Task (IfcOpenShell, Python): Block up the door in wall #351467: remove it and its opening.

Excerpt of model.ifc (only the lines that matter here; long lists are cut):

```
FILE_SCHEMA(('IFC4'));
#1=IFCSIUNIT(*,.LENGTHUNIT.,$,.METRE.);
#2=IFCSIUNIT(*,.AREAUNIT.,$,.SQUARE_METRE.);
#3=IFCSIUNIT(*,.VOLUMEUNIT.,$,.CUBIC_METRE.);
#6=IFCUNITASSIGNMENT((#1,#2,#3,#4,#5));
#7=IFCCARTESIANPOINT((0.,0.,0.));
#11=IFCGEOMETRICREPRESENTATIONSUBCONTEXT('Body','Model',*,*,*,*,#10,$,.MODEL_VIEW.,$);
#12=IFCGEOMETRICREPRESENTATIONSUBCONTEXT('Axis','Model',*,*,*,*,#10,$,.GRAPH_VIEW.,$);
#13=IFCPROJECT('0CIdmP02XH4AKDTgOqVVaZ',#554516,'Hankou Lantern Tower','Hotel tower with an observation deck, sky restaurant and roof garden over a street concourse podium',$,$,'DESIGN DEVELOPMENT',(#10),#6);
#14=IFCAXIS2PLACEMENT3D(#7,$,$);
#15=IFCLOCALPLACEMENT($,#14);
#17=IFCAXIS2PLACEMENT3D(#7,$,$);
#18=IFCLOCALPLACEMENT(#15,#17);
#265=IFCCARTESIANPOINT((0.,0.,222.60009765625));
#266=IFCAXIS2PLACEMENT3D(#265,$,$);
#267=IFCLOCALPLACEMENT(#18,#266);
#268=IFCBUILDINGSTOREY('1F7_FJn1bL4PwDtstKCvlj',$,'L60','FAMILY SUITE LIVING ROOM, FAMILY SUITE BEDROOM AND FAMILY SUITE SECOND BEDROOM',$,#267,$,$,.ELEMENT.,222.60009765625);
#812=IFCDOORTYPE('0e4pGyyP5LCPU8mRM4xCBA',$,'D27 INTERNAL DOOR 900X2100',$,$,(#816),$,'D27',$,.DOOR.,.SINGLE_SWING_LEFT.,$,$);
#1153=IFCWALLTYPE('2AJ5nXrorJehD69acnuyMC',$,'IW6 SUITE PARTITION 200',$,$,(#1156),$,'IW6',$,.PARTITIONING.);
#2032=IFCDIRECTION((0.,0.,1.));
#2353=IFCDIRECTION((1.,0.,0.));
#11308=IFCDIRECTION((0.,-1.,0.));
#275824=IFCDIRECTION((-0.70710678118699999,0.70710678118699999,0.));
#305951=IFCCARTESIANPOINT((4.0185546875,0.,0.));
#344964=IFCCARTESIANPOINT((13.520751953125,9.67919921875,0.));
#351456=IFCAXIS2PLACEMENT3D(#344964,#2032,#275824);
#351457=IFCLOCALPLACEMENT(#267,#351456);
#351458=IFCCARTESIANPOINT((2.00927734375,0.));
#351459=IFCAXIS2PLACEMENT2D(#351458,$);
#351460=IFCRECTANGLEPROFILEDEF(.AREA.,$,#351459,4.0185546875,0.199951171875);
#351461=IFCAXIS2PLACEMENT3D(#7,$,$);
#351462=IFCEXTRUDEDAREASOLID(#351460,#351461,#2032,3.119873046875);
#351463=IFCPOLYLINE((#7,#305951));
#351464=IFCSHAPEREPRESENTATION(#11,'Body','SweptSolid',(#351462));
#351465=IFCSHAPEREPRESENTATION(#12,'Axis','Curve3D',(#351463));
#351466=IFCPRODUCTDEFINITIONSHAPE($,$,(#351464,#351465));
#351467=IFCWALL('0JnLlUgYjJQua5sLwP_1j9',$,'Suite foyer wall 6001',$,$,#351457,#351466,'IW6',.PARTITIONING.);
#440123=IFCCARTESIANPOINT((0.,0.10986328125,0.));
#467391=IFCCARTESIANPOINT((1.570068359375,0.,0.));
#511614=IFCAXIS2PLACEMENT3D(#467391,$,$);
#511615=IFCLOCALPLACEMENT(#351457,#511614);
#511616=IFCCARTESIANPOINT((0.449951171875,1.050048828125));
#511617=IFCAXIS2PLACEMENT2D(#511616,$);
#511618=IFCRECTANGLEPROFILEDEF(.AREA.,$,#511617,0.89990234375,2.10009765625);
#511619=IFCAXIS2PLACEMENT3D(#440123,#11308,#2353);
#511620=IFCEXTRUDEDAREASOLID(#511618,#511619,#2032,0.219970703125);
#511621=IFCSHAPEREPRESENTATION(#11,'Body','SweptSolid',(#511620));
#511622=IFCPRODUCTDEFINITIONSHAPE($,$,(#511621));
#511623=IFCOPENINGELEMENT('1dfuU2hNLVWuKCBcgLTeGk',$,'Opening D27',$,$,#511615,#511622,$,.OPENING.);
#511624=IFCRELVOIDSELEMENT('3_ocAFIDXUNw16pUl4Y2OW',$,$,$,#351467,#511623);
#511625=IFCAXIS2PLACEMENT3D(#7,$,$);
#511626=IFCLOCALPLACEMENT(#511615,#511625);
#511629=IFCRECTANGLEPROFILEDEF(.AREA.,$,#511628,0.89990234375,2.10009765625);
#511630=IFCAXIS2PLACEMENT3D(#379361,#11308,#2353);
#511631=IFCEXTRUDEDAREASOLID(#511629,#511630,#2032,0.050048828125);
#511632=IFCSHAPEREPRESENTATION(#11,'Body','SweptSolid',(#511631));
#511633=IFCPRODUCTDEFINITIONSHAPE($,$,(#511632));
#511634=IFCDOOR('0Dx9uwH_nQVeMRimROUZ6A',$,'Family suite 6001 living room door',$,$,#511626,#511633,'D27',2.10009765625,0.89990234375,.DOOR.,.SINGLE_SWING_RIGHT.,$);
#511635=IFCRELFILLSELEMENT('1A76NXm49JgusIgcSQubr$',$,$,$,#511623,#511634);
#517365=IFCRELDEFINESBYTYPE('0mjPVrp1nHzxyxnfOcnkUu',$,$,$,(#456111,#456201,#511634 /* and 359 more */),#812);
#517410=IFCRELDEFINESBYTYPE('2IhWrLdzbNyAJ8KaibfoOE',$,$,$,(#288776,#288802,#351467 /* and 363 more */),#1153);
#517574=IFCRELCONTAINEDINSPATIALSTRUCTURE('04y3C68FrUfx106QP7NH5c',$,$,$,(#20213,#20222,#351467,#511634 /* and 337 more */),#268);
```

```python
import ifcopenshell
import ifcopenshell.api.feature
import ifcopenshell.api.root
import ifcopenshell.geom
import ifcopenshell.util.shape

model = ifcopenshell.open("model.ifc")
settings = ifcopenshell.geom.settings()


def volume(element):
    """Net volume in cubic metres, openings subtracted."""
    shape = ifcopenshell.geom.create_shape(settings, element)
    return ifcopenshell.util.shape.get_volume(shape.geometry)


door = model.by_guid("0Dx9uwH_nQVeMRimROUZ6A")
opening = door.FillsVoids[0].RelatingOpeningElement
wall = opening.VoidsElements[0].RelatingBuildingElement
before = volume(wall)

ifcopenshell.api.root.remove_product(model, product=door)
ifcopenshell.api.feature.remove_feature(model, feature=opening)

after = volume(wall)

print(f"wall volume {before:.3f} -> {after:.3f} m3")

model.write("model_updated.ifc")
```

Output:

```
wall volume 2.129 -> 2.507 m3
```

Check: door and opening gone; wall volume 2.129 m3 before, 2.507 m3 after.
